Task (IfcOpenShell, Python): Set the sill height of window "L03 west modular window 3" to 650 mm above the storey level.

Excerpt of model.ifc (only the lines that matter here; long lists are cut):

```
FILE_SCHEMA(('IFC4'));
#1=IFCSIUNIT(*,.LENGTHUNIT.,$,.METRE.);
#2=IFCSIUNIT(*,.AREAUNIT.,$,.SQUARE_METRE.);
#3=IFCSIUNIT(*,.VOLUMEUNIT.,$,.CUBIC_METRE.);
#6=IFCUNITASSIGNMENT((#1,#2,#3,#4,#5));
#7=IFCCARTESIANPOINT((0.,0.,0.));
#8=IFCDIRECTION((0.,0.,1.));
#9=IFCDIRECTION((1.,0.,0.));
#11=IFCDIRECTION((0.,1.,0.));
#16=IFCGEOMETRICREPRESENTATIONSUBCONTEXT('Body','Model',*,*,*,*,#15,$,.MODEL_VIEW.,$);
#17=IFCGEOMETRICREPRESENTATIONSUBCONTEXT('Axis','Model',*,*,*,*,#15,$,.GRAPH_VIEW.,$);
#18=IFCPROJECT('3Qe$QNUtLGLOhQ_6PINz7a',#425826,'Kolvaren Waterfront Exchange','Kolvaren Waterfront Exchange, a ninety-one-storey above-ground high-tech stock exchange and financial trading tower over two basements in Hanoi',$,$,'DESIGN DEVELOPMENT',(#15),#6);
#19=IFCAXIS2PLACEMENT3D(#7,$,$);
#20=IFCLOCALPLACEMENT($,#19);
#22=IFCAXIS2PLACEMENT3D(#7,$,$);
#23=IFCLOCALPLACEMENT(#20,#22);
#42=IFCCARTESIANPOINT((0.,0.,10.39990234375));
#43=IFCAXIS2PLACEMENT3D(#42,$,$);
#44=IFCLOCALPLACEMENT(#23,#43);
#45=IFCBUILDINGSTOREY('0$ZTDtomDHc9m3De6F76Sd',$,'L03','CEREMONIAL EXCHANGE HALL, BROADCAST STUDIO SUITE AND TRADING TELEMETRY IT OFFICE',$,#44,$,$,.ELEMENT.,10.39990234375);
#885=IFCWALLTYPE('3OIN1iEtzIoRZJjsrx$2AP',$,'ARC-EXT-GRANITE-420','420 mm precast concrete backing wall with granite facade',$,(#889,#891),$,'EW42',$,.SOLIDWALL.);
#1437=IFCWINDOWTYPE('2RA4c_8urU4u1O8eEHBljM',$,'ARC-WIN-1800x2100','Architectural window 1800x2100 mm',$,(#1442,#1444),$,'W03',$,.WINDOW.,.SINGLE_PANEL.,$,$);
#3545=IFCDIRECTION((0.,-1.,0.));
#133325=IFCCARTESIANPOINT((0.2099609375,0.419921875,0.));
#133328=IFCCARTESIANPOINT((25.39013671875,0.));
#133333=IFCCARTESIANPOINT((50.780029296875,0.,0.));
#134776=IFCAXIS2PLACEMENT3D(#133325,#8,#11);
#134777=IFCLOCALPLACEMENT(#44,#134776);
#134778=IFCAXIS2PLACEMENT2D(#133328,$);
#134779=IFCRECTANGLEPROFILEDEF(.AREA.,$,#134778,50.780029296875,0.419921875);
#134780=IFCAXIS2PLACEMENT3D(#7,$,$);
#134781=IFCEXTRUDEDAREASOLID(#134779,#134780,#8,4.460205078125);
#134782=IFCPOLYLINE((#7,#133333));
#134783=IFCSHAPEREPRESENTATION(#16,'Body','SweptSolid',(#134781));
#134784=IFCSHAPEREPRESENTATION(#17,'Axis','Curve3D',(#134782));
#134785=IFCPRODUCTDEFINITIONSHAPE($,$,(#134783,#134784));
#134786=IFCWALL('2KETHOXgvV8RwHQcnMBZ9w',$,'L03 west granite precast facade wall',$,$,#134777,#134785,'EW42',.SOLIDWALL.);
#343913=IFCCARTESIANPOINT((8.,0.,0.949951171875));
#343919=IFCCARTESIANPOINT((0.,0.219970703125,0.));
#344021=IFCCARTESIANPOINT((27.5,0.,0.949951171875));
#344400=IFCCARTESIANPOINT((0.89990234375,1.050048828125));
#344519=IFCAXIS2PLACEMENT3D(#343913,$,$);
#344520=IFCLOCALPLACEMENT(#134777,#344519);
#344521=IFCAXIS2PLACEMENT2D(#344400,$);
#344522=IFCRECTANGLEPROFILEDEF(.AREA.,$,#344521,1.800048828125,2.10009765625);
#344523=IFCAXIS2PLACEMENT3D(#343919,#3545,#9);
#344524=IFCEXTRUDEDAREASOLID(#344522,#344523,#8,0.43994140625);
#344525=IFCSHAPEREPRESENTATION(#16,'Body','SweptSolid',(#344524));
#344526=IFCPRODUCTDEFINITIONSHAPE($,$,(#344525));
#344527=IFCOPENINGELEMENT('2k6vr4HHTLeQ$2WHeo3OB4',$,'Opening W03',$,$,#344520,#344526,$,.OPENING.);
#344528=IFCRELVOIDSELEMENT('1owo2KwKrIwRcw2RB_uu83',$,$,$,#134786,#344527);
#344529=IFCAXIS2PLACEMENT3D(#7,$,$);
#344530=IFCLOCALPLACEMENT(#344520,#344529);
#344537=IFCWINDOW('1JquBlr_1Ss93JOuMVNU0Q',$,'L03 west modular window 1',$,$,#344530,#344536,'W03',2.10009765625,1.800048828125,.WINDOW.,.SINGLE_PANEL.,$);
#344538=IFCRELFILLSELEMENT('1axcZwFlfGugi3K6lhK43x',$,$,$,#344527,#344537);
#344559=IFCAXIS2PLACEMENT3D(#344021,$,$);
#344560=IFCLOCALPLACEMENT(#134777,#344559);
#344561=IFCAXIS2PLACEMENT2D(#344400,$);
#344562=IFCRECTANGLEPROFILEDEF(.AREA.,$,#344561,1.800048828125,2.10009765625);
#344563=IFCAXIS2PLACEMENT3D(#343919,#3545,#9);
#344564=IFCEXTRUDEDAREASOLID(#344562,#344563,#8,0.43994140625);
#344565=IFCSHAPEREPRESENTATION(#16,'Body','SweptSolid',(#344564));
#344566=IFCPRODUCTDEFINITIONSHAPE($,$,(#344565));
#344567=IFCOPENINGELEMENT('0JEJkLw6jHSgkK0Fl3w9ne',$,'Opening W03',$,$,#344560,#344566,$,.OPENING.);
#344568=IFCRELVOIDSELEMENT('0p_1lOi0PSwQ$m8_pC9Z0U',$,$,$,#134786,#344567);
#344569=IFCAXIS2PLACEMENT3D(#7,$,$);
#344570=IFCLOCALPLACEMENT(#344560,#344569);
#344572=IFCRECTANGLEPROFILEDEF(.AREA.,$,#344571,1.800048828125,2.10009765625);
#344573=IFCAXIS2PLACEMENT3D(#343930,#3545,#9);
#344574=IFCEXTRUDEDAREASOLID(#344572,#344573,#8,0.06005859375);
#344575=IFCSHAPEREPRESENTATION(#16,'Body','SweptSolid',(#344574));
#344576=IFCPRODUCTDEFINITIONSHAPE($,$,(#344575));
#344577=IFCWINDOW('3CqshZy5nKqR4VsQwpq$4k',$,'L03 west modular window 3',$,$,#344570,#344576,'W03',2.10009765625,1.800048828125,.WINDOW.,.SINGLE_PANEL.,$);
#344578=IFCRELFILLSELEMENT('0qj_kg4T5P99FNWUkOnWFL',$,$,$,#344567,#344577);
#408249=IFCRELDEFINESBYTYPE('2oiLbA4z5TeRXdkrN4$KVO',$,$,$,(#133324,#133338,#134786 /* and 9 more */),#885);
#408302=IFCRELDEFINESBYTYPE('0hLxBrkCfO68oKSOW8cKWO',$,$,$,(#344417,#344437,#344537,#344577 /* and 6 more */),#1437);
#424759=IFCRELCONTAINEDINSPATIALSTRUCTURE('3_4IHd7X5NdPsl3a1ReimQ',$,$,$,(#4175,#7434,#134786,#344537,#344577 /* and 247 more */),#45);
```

```python
import numpy as np
import ifcopenshell
import ifcopenshell.api.geometry
import ifcopenshell.geom
import ifcopenshell.util.element
import ifcopenshell.util.placement
import ifcopenshell.util.shape
import ifcopenshell.util.unit

model = ifcopenshell.open("model.ifc")
unit_scale = ifcopenshell.util.unit.calculate_unit_scale(model)

window = model.by_guid("3CqshZy5nKqR4VsQwpq$4k")
opening = window.FillsVoids[0].RelatingOpeningElement
storey = ifcopenshell.util.element.get_container(window, ifc_class="IfcBuildingStorey")
level = ifcopenshell.util.placement.get_local_placement(storey.ObjectPlacement)[2, 3]

# The opening's origin need not be at the sill, so measure its lowest point.
shape = ifcopenshell.geom.create_shape(ifcopenshell.geom.settings(), opening)
bottom = ifcopenshell.util.shape.get_shape_bottom_elevation(shape, shape.geometry) / unit_scale
dz = level + 0.65 - bottom

shift = np.array([0.0, 0.0, dz])
# The window is placed relative to its opening, so it follows when the opening moves.
matrix = ifcopenshell.util.placement.get_local_placement(opening.ObjectPlacement)
matrix[:3, 3] += shift
ifcopenshell.api.geometry.edit_object_placement(
    model, product=opening, matrix=matrix, is_si=False, should_transform_children=True
)

print(f"moved by {dz * unit_scale:+.3f} m")

model.write("model-out.ifc")
```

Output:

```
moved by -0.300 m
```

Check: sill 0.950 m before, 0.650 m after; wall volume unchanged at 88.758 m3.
